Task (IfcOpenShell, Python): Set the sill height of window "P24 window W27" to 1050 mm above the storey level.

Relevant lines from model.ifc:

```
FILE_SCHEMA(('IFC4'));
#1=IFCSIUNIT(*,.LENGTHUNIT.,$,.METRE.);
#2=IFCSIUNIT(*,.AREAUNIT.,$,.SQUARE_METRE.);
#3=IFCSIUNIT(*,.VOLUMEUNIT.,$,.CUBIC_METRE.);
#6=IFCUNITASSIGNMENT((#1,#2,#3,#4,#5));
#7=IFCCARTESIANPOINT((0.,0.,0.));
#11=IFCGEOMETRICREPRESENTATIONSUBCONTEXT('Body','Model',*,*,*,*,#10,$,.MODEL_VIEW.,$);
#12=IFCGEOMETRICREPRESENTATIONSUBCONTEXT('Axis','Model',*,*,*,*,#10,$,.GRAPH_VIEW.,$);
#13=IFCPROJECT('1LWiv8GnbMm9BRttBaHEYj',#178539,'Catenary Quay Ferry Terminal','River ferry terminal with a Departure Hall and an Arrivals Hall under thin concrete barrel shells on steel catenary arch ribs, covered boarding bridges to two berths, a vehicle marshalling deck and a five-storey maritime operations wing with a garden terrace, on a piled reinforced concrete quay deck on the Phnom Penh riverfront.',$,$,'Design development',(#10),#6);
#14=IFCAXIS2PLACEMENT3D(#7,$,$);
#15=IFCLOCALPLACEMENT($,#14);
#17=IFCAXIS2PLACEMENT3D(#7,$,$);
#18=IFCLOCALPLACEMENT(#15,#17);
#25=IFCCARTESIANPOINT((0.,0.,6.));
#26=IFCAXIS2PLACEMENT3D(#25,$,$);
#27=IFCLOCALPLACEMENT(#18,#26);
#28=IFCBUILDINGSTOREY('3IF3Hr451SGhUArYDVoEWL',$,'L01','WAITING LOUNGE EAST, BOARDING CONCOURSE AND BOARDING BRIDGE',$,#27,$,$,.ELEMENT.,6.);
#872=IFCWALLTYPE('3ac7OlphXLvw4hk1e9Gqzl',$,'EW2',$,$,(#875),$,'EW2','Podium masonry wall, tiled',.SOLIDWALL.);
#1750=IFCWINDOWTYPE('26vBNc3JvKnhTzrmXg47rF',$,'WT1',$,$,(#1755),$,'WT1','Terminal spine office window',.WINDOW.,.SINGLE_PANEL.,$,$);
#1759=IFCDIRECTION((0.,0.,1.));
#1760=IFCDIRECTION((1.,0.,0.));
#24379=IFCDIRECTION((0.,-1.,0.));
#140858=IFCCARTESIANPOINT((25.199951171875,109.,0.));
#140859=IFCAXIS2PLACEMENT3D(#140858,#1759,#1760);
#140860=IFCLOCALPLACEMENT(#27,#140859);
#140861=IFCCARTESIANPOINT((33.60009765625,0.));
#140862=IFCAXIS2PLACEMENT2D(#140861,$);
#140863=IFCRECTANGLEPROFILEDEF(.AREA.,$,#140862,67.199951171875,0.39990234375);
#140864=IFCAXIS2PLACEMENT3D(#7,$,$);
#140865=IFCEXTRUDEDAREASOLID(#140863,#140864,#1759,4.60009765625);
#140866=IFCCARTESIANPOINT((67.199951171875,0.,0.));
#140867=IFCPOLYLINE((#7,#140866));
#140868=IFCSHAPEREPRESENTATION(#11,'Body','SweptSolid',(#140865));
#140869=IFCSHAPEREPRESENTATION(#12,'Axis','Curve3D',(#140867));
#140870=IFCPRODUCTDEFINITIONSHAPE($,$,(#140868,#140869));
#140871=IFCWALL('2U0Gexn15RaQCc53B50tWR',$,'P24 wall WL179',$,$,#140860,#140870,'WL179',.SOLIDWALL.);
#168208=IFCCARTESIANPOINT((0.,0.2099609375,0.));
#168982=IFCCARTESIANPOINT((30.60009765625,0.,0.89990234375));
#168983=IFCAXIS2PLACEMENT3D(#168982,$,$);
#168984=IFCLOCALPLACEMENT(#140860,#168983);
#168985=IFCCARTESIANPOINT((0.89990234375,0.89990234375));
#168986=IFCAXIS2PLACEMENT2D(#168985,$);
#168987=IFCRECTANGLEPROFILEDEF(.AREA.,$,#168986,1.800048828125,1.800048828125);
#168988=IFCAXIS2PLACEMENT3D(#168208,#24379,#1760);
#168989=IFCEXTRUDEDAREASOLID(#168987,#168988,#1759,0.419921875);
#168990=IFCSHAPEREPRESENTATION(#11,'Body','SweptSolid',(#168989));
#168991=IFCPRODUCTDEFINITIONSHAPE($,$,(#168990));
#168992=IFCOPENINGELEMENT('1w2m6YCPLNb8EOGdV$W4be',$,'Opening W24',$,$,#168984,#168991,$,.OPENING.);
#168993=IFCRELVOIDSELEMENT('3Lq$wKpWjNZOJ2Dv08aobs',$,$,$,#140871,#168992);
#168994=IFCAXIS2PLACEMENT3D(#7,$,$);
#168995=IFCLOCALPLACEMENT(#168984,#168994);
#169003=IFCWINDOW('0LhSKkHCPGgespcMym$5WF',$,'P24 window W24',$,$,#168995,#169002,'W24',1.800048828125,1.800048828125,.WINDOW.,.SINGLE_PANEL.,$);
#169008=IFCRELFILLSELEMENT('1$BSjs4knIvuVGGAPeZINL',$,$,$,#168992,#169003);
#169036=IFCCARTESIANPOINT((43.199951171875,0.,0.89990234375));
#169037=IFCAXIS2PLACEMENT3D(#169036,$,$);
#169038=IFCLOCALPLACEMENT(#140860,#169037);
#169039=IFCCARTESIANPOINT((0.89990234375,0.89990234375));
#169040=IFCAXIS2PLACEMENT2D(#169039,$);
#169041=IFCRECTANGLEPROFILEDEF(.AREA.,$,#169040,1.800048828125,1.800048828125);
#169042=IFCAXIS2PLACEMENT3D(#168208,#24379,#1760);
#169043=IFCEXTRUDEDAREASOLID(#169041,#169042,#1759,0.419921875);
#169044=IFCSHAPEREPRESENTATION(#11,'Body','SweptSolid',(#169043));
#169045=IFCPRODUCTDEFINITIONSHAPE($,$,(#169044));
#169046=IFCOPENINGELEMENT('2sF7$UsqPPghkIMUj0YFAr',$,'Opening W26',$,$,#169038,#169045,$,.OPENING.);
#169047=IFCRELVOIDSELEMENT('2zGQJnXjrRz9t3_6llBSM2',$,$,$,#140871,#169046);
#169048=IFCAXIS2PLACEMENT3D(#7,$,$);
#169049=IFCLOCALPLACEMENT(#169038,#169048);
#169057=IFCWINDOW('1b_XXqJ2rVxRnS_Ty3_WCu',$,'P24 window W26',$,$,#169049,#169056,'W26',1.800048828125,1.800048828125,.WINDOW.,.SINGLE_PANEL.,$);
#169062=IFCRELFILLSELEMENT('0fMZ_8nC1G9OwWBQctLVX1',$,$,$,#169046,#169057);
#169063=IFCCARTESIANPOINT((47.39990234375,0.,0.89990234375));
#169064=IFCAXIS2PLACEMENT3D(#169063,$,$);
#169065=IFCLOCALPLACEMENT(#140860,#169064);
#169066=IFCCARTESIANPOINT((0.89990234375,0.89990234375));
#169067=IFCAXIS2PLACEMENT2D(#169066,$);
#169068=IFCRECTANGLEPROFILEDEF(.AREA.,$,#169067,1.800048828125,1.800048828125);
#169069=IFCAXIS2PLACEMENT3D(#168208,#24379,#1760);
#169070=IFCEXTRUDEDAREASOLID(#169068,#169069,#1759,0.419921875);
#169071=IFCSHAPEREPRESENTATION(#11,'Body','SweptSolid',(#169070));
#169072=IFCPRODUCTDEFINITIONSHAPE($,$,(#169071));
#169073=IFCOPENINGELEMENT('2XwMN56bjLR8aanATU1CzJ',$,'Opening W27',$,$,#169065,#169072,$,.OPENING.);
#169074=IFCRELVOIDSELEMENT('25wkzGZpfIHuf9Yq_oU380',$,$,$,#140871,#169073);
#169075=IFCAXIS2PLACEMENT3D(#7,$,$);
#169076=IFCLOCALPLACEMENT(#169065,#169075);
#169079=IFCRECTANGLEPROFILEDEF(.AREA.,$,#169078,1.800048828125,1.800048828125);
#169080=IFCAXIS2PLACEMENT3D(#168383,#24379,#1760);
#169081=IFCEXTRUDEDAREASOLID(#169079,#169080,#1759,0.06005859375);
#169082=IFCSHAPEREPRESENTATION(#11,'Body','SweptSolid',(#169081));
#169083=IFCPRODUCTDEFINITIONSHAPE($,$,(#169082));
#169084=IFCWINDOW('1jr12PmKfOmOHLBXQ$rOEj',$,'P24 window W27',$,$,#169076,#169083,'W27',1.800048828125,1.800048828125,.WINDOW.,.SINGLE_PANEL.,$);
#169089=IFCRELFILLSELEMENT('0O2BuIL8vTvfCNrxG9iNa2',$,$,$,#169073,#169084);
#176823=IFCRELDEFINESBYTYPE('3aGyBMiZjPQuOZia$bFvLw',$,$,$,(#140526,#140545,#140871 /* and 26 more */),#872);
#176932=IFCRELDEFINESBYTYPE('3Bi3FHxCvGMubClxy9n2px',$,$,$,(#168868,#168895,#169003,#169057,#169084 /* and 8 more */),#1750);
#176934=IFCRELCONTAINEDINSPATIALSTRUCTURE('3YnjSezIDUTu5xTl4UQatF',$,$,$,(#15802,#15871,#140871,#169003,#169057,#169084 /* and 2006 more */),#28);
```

```python
import numpy as np
import ifcopenshell
import ifcopenshell.api.geometry
import ifcopenshell.geom
import ifcopenshell.util.element
import ifcopenshell.util.placement
import ifcopenshell.util.shape
import ifcopenshell.util.unit

model = ifcopenshell.open("model.ifc")
unit_scale = ifcopenshell.util.unit.calculate_unit_scale(model)

window = model.by_guid("1jr12PmKfOmOHLBXQ$rOEj")
opening = window.FillsVoids[0].RelatingOpeningElement
storey = ifcopenshell.util.element.get_container(window, ifc_class="IfcBuildingStorey")
level = ifcopenshell.util.placement.get_local_placement(storey.ObjectPlacement)[2, 3]

# The opening's origin need not be at the sill, so measure its lowest point.
shape = ifcopenshell.geom.create_shape(ifcopenshell.geom.settings(), opening)
bottom = ifcopenshell.util.shape.get_shape_bottom_elevation(shape, shape.geometry) / unit_scale
dz = level + 1.05 - bottom

shift = np.array([0.0, 0.0, dz])
# The window is placed relative to its opening, so it follows when the opening moves.
matrix = ifcopenshell.util.placement.get_local_placement(opening.ObjectPlacement)
matrix[:3, 3] += shift
ifcopenshell.api.geometry.edit_object_placement(
    model, product=opening, matrix=matrix, is_si=False, should_transform_children=True
)

print(f"moved by {dz * unit_scale:+.3f} m")

model.write("model_rev.ifc")
```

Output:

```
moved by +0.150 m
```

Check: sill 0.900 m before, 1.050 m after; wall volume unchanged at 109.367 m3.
